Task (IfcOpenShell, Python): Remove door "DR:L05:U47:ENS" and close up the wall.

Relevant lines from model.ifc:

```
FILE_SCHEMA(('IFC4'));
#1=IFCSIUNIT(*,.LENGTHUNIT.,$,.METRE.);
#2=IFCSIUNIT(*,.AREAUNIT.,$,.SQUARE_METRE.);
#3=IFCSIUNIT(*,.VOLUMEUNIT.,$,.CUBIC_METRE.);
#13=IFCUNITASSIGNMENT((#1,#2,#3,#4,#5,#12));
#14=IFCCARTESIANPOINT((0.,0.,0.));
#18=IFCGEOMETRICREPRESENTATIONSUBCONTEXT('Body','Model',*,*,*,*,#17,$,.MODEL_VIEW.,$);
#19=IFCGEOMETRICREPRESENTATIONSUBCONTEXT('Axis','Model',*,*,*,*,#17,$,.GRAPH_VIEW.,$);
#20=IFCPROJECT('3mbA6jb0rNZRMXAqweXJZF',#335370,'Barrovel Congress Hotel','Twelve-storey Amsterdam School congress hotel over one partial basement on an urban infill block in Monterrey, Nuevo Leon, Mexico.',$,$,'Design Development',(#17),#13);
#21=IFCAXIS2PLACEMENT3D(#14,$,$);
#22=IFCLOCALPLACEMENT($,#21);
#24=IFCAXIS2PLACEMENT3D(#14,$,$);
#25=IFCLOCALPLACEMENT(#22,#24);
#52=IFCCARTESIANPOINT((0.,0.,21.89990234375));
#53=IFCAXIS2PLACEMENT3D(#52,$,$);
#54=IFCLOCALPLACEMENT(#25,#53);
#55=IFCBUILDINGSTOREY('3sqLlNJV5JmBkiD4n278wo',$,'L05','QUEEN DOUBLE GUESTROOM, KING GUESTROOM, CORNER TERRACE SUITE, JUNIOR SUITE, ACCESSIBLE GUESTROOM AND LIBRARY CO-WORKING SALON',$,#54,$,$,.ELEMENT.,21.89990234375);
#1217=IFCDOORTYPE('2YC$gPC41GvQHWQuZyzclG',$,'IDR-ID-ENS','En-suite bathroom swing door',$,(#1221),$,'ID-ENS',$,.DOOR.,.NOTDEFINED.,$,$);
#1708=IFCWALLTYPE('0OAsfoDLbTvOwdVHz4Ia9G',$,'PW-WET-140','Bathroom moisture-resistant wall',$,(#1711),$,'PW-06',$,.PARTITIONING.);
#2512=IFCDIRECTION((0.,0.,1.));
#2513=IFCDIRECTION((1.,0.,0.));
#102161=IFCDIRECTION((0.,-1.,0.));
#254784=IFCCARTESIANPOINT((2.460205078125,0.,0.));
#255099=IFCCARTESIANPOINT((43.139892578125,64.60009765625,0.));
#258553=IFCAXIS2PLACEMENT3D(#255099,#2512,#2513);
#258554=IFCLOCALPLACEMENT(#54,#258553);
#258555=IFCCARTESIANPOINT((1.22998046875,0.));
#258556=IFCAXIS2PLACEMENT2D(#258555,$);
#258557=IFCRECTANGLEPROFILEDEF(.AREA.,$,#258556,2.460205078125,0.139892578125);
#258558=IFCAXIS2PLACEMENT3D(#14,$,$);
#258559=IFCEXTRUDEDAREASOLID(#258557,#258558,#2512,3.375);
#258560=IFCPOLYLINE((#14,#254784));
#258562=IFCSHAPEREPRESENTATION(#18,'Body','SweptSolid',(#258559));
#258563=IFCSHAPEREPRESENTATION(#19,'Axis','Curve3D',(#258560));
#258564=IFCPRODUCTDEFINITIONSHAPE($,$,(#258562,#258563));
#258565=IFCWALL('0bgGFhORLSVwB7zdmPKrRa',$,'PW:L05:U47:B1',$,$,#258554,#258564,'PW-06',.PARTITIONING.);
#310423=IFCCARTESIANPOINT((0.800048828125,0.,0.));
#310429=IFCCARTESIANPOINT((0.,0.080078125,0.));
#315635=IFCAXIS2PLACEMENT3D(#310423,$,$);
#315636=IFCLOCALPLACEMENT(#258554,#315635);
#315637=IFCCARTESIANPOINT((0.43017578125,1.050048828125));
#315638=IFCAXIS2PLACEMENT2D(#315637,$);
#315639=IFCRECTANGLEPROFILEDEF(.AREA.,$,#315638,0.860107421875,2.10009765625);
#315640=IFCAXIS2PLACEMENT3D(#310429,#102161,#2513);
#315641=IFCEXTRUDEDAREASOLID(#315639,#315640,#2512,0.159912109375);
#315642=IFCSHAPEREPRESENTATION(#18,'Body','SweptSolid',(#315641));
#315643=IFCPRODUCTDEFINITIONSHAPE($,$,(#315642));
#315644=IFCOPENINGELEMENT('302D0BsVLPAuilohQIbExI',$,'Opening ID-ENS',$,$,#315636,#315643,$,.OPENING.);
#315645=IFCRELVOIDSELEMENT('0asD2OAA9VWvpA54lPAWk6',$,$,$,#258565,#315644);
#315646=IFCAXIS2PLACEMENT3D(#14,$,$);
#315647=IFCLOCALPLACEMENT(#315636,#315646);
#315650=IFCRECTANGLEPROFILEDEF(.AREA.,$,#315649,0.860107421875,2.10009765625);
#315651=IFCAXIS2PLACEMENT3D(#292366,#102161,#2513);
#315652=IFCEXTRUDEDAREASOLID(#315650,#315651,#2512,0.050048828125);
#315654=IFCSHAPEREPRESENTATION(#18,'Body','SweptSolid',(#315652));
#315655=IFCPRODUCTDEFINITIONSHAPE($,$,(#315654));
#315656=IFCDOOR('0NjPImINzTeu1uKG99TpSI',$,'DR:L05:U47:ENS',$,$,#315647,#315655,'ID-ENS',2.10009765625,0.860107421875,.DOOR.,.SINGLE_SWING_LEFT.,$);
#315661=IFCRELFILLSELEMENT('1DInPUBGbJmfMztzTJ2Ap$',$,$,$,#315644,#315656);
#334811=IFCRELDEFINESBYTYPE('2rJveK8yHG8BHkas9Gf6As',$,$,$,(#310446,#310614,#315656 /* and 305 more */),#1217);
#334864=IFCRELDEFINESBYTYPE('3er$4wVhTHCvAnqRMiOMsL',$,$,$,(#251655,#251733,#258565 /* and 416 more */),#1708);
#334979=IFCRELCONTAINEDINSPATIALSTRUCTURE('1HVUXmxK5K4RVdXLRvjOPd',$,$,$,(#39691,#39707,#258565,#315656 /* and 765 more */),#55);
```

```python
import ifcopenshell
import ifcopenshell.api.feature
import ifcopenshell.api.root
import ifcopenshell.geom
import ifcopenshell.util.shape

model = ifcopenshell.open("model.ifc")
settings = ifcopenshell.geom.settings()


def volume(element):
    """Net volume in cubic metres, openings subtracted."""
    shape = ifcopenshell.geom.create_shape(settings, element)
    return ifcopenshell.util.shape.get_volume(shape.geometry)


door = model.by_guid("0NjPImINzTeu1uKG99TpSI")
opening = door.FillsVoids[0].RelatingOpeningElement
wall = opening.VoidsElements[0].RelatingBuildingElement
before = volume(wall)

ifcopenshell.api.root.remove_product(model, product=door)
ifcopenshell.api.feature.remove_feature(model, feature=opening)

after = volume(wall)

print(f"wall volume {before:.3f} -> {after:.3f} m3")

model.write("model_rev.ifc")
```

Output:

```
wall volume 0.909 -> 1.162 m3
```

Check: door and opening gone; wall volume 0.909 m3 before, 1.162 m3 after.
